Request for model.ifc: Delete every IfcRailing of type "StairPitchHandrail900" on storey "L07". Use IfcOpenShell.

First a look at what the model holds.

```python
import ifcopenshell
import ifcopenshell.util.element

model = ifcopenshell.open("model.ifc")
print(model.schema)
storey = next(s for s in model.by_type("IfcBuildingStorey") if s.Name == "L07")
railings = [e for e in ifcopenshell.util.element.get_decomposition(storey) if e.is_a("IfcRailing")]
seen = {}
for e in railings:
    element_type = ifcopenshell.util.element.get_type(e)
    name = element_type.Name if element_type not in (None, e) else None
    seen[name] = seen.get(name, 0) + 1
for name, count in sorted(seen.items(), key=str):
    print(count, "x", name)
```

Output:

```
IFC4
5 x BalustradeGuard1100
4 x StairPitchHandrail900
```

```python
import ifcopenshell
import ifcopenshell.api.root
import ifcopenshell.util.element

model = ifcopenshell.open("model.ifc")

storey = next(s for s in model.by_type("IfcBuildingStorey") if s.Name == "L07")
railings = [e for e in ifcopenshell.util.element.get_decomposition(storey) if e.is_a("IfcRailing")]
targets = [e for e in railings if (t := ifcopenshell.util.element.get_type(e)) not in (None, e) and t.Name == "StairPitchHandrail900"]

for e in targets:
    ifcopenshell.api.root.remove_product(model, product=e)
print(len(targets), "removed")

model.write("model_v2.ifc")
```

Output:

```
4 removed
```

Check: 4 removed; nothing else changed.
